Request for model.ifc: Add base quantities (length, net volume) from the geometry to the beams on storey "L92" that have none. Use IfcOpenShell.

First a look at what the model holds.

```python
import ifcopenshell
import ifcopenshell.util.element
import ifcopenshell.util.unit

model = ifcopenshell.open("model.ifc")
print(model.schema)
for unit_type in ("LENGTHUNIT", "AREAUNIT", "VOLUMEUNIT"):
    print(unit_type, ifcopenshell.util.unit.calculate_unit_scale(model, unit_type))
storey = next(s for s in model.by_type("IfcBuildingStorey") if s.Name == "L92")
beams = [e for e in ifcopenshell.util.element.get_decomposition(storey) if e.is_a("IfcBeam")]
for e in sorted(beams, key=lambda e: e.id()):
    print(e.id(), e.is_a(), e.Name, list(ifcopenshell.util.element.get_psets(e, qtos_only=True)), sep=" | ")
```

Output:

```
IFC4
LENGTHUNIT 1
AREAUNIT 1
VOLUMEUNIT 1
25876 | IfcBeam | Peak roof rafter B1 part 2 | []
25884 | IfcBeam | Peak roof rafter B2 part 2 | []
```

```python
import ifcopenshell
import ifcopenshell.api.pset
import ifcopenshell.geom
import ifcopenshell.util.element
import ifcopenshell.util.shape
import ifcopenshell.util.unit

model = ifcopenshell.open("model.ifc")
unit_scale = ifcopenshell.util.unit.calculate_unit_scale(model)
volume_scale = ifcopenshell.util.unit.calculate_unit_scale(model, "VOLUMEUNIT")
settings = ifcopenshell.geom.settings()

storey = next(s for s in model.by_type("IfcBuildingStorey") if s.Name == "L92")
beams = [e for e in ifcopenshell.util.element.get_decomposition(storey) if e.is_a("IfcBeam")]

for e in sorted(beams, key=lambda e: e.id()):
    if ifcopenshell.util.element.get_psets(e, qtos_only=True, should_inherit=False):
        continue
    # Geometry comes back in metres, in the element's own axes.
    shape = ifcopenshell.geom.create_shape(settings, e)
    values = {
        "Length": ifcopenshell.util.shape.get_max_xyz(shape.geometry) / unit_scale,
        "NetVolume": ifcopenshell.util.shape.get_volume(shape.geometry) / volume_scale,
    }
    qto = ifcopenshell.api.pset.add_qto(model, product=e, name="Qto_BeamBaseQuantities")
    ifcopenshell.api.pset.edit_qto(model, qto=qto, properties=values)
    print(e.id(), {k: round(v, 3) for k, v in values.items()})

model.write("model_edited.ifc")
```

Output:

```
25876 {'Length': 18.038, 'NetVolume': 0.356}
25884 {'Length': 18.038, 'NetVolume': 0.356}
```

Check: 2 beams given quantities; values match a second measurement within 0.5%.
